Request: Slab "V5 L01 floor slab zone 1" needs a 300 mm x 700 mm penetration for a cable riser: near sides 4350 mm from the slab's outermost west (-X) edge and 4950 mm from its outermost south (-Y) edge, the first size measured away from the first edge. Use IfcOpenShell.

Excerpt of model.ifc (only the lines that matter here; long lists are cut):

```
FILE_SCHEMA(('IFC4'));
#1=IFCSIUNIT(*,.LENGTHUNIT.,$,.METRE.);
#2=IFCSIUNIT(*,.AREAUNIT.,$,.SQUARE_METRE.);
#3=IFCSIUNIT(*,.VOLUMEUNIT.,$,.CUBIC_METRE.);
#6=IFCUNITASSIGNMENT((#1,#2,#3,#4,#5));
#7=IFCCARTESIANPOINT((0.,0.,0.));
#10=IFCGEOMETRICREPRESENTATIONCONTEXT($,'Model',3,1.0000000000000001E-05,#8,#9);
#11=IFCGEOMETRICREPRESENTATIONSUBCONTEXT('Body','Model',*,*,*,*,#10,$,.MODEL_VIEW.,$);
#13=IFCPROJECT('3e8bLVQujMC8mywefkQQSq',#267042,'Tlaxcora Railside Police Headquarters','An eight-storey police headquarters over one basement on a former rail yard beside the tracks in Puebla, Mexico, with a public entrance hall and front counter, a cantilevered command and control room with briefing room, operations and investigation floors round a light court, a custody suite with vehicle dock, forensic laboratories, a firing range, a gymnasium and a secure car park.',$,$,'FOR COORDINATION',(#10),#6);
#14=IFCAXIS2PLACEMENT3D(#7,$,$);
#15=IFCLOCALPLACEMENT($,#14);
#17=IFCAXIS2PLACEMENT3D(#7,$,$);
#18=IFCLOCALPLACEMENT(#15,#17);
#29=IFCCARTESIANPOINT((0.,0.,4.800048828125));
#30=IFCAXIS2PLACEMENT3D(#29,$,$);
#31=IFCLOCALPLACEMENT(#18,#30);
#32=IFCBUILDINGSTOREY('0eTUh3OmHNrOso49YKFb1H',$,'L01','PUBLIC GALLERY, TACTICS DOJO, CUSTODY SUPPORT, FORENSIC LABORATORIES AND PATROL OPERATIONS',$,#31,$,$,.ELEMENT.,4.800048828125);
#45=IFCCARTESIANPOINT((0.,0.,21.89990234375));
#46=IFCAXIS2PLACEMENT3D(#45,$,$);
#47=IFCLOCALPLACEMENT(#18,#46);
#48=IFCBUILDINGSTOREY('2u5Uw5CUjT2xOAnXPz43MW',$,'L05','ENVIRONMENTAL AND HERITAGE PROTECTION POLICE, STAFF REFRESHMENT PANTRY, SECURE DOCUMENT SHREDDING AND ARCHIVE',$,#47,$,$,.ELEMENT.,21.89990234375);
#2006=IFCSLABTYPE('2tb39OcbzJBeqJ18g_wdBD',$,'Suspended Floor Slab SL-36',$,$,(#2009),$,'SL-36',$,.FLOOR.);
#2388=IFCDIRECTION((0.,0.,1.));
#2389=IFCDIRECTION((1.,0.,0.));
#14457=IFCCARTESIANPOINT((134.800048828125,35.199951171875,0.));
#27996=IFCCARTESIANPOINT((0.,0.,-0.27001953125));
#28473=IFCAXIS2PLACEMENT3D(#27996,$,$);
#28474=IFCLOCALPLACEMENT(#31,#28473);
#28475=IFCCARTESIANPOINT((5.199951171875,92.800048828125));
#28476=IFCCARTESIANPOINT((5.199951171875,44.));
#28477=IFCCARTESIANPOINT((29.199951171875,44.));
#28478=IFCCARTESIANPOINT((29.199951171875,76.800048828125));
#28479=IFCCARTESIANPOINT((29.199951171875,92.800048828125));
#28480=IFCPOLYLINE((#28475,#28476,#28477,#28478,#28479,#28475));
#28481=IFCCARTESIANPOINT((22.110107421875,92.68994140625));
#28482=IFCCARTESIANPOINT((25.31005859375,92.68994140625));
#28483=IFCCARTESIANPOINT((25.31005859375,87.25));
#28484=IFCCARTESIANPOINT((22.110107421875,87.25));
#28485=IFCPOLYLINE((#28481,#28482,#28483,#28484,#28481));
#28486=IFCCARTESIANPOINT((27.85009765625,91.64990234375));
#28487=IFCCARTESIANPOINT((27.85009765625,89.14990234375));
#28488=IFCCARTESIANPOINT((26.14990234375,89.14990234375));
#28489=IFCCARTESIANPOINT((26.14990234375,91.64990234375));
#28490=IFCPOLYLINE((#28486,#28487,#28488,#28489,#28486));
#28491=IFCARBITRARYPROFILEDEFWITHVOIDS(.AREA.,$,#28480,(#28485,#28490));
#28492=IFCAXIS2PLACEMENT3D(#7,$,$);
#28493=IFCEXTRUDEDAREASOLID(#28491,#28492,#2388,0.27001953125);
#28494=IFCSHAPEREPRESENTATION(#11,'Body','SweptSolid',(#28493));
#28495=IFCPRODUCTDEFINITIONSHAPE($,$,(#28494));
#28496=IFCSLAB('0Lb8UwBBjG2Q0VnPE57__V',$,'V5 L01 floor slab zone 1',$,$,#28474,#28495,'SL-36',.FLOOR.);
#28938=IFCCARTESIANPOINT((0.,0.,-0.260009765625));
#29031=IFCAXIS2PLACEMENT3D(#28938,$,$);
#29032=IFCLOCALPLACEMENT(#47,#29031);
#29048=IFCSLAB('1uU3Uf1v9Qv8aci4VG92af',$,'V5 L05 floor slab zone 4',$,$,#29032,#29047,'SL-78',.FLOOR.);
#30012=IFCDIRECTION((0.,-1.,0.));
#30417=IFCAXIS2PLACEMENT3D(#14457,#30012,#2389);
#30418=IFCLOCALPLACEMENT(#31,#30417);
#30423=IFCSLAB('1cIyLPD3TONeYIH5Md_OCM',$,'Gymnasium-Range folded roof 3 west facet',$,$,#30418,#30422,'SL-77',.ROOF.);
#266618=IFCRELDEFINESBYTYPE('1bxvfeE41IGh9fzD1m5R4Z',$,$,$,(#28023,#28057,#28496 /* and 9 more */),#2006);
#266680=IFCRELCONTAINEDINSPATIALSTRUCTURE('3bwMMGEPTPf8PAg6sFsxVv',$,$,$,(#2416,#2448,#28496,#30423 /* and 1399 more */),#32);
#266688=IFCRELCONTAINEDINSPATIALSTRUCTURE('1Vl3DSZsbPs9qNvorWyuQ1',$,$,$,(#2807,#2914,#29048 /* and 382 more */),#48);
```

```python
import numpy as np
import ifcopenshell
import ifcopenshell.api.feature
import ifcopenshell.api.geometry
import ifcopenshell.api.root
import ifcopenshell.geom
import ifcopenshell.util.placement
import ifcopenshell.util.representation
import ifcopenshell.util.shape
import ifcopenshell.util.unit

model = ifcopenshell.open("model.ifc")
unit_scale = ifcopenshell.util.unit.calculate_unit_scale(model)
settings = ifcopenshell.geom.settings()


def volume(element):
    """Net volume in cubic metres, openings subtracted."""
    shape = ifcopenshell.geom.create_shape(settings, element)
    return ifcopenshell.util.shape.get_volume(shape.geometry)


slab = model.by_id(28496)
before = volume(slab)

# Extent in the slab's own axes, in metres. The edges named are its -X and -Y sides.
slab_shape = ifcopenshell.geom.create_shape(settings, slab)
vertices = ifcopenshell.util.shape.get_vertices(slab_shape.geometry)
x_min, y_min, bottom = vertices.min(axis=0)
top = vertices[:, 2].max()

opening = ifcopenshell.api.root.create_entity(model, ifc_class="IfcOpeningElement", name="Cable riser opening", predefined_type="OPENING")
context = ifcopenshell.util.representation.get_context(model, "Model", "Body", "MODEL_VIEW")
width, depth = 0.3, 0.7
outline = [(0.0, 0.0), (width, 0.0), (width, depth), (0.0, depth), (0.0, 0.0)]
# Overshoot both faces by 50 mm so the cut is clean.
shape = ifcopenshell.api.geometry.add_slab_representation(
    model, context=context, depth=top - bottom + 0.1, polyline=outline
)
ifcopenshell.api.geometry.assign_representation(model, product=opening, representation=shape)

matrix = ifcopenshell.util.placement.get_local_placement(slab.ObjectPlacement)
matrix[:, 3] = matrix @ np.append(np.array([x_min + 4.35, y_min + 4.95, bottom - 0.05]) / unit_scale, 1.0)
ifcopenshell.api.geometry.edit_object_placement(model, product=opening, matrix=matrix, is_si=False)
ifcopenshell.api.feature.add_feature(model, feature=opening, element=slab)

after = volume(slab)

print(f"slab volume {before:.3f} -> {after:.3f} m3")

model.write("model_edited.ifc")
```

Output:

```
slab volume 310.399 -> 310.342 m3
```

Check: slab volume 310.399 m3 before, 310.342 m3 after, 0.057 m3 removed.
